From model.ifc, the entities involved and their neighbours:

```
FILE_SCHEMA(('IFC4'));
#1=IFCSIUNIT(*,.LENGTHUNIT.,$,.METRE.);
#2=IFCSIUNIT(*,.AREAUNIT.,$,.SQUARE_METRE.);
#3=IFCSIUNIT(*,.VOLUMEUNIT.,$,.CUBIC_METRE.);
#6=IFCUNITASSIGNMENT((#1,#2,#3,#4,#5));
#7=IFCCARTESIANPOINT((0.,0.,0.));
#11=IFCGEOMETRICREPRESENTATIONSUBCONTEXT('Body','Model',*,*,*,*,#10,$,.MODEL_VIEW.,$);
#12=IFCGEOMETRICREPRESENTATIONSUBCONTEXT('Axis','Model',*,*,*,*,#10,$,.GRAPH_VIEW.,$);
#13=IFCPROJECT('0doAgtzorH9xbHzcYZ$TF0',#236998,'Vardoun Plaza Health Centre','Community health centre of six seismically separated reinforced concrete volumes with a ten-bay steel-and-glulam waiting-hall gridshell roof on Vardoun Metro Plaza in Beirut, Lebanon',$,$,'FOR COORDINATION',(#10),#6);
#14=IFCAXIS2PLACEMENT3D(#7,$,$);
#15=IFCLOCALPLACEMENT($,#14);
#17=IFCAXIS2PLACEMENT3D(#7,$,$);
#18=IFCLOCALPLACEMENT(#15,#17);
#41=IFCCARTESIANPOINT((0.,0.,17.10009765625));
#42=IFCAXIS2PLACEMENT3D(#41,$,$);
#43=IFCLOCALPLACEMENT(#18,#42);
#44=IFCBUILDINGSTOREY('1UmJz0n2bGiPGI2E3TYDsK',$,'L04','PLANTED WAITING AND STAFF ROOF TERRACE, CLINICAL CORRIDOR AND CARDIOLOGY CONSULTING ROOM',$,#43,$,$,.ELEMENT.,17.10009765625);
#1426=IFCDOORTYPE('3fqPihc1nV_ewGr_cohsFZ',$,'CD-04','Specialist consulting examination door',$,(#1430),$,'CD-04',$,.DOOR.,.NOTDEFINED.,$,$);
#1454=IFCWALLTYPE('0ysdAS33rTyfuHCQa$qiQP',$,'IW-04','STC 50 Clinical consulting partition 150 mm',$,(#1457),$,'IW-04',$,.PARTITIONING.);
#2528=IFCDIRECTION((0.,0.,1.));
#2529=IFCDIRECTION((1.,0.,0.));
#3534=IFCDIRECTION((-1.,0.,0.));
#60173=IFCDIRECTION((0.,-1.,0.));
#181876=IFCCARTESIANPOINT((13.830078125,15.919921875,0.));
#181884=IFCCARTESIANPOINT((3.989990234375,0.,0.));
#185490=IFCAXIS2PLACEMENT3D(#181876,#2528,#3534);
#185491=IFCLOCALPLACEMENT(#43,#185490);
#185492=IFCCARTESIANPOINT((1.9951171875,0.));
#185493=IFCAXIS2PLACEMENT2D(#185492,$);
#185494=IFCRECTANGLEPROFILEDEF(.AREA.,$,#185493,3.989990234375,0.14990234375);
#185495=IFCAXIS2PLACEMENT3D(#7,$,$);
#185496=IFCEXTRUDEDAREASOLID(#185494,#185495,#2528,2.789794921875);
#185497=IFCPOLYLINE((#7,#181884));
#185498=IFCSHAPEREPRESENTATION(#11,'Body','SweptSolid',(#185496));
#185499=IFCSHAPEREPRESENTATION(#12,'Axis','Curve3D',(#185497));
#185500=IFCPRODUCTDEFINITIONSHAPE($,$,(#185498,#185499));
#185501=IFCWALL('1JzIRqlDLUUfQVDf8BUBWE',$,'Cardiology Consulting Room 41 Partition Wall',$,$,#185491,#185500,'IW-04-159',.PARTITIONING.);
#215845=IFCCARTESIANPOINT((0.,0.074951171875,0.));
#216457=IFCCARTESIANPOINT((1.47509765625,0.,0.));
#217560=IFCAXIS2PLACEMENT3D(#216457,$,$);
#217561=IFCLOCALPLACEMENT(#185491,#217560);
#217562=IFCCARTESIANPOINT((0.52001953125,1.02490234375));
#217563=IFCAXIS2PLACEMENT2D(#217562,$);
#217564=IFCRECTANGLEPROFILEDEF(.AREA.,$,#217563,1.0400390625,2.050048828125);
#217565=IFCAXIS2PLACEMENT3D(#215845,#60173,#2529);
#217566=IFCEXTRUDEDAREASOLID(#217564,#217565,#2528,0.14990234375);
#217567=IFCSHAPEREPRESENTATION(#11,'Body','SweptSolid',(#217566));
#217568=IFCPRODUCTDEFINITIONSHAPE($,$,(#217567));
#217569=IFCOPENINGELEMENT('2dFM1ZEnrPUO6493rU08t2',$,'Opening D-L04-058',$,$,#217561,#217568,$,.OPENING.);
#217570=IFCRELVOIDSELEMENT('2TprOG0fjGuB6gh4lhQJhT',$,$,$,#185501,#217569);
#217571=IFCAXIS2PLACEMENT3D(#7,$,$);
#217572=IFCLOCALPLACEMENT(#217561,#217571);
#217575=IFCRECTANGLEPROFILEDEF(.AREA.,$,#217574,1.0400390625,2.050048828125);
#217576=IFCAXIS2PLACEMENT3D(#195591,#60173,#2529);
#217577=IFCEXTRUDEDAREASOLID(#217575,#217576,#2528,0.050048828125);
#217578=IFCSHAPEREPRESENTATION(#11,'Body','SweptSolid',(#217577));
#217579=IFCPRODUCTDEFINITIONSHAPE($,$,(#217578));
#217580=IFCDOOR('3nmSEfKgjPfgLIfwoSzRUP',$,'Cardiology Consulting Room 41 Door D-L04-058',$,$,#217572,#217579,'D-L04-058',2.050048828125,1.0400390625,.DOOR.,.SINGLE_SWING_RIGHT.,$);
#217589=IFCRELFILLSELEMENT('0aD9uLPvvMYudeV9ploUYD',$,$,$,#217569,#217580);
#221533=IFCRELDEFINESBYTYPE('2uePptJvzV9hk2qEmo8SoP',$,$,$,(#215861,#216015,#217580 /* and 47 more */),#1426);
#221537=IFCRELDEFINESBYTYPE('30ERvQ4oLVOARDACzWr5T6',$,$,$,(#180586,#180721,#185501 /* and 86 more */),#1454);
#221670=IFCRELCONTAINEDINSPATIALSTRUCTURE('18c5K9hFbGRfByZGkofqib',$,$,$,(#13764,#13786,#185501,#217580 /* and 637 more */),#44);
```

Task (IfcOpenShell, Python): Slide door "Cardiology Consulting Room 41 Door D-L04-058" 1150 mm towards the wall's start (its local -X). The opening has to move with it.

```python
import ifcopenshell
import ifcopenshell.api.geometry
import ifcopenshell.util.placement

model = ifcopenshell.open("model.ifc")

door = model.by_guid("3nmSEfKgjPfgLIfwoSzRUP")
opening = door.FillsVoids[0].RelatingOpeningElement
wall = opening.VoidsElements[0].RelatingBuildingElement

wall_matrix = ifcopenshell.util.placement.get_local_placement(wall.ObjectPlacement)
shift = wall_matrix[:3, 0] * -1.15
before = ifcopenshell.util.placement.get_local_placement(door.ObjectPlacement)[:3, 3].copy()

# The door is placed relative to its opening, so it follows when the opening moves.
matrix = ifcopenshell.util.placement.get_local_placement(opening.ObjectPlacement)
matrix[:3, 3] += shift
ifcopenshell.api.geometry.edit_object_placement(
    model, product=opening, matrix=matrix, is_si=False, should_transform_children=True
)

after = ifcopenshell.util.placement.get_local_placement(door.ObjectPlacement)[:3, 3]
print("door moved by", (after - before).round(3) + 0.0)

model.write("model_edited.ifc")
```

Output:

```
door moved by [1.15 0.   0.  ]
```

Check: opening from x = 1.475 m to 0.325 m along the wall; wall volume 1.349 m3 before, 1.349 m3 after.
